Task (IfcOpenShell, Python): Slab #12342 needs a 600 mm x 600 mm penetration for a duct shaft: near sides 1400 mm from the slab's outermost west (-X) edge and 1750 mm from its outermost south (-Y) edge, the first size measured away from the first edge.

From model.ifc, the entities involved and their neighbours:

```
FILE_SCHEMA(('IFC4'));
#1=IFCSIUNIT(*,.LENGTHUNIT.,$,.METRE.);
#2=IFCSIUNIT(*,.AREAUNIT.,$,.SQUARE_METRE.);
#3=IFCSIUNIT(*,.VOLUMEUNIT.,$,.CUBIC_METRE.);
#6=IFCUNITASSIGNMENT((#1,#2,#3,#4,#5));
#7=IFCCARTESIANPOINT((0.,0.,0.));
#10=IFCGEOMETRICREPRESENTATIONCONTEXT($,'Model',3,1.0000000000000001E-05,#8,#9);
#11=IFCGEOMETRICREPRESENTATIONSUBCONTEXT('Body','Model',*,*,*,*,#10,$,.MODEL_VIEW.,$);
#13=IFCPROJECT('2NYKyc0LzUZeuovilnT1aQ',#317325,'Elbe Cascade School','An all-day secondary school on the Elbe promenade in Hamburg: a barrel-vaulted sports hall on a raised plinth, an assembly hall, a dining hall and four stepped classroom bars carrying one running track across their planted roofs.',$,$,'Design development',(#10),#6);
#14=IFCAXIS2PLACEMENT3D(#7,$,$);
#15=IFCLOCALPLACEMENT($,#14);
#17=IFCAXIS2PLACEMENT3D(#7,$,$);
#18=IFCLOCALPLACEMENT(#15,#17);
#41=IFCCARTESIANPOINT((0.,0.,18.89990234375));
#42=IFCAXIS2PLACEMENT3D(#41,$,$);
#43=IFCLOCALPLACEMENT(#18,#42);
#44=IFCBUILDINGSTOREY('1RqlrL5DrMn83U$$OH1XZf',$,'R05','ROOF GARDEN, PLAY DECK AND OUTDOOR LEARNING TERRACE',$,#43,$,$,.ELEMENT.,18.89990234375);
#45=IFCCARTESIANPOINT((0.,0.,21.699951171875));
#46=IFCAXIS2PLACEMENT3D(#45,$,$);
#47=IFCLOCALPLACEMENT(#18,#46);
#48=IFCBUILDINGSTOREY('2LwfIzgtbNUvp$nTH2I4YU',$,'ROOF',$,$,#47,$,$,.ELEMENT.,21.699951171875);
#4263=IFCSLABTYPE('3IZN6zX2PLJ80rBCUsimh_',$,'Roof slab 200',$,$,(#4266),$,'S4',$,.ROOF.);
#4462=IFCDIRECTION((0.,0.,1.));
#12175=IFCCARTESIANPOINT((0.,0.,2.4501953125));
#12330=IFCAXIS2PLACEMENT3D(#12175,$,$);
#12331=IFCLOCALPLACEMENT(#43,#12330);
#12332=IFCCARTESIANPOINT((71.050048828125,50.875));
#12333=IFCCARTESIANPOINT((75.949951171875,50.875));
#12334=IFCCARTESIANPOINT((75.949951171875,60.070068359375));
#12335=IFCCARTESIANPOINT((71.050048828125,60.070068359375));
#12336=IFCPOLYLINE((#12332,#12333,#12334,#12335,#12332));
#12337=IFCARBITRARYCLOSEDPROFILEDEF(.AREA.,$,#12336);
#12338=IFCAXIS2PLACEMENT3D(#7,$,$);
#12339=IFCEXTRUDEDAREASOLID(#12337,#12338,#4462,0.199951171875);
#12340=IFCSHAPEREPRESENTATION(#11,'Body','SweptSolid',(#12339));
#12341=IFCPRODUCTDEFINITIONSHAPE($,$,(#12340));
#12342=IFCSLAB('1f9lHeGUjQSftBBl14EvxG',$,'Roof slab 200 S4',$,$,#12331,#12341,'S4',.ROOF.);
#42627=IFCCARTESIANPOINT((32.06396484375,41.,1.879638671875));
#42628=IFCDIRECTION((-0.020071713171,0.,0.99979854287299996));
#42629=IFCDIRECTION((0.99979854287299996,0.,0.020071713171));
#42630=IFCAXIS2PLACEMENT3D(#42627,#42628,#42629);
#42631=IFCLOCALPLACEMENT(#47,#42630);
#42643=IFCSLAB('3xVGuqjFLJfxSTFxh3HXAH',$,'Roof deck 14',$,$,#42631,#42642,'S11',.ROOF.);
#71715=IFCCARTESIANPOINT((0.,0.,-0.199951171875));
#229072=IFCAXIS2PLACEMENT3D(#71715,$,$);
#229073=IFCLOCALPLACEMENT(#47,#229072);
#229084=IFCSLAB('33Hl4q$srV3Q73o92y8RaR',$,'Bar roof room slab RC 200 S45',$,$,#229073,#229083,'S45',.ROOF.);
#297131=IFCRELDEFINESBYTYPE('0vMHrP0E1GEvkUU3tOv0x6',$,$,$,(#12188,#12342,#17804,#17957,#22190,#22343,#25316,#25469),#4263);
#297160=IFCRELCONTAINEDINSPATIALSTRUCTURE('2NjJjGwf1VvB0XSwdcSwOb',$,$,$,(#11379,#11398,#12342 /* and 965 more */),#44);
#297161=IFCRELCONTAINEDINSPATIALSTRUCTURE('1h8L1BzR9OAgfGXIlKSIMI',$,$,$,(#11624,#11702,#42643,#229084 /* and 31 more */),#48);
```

```python
import numpy as np
import ifcopenshell
import ifcopenshell.api.feature
import ifcopenshell.api.geometry
import ifcopenshell.api.root
import ifcopenshell.geom
import ifcopenshell.util.placement
import ifcopenshell.util.representation
import ifcopenshell.util.shape
import ifcopenshell.util.unit

model = ifcopenshell.open("model.ifc")
unit_scale = ifcopenshell.util.unit.calculate_unit_scale(model)
settings = ifcopenshell.geom.settings()


def volume(element):
    """Net volume in cubic metres, openings subtracted."""
    shape = ifcopenshell.geom.create_shape(settings, element)
    return ifcopenshell.util.shape.get_volume(shape.geometry)


slab = model.by_guid("1f9lHeGUjQSftBBl14EvxG")
before = volume(slab)

# Extent in the slab's own axes, in metres. The edges named are its -X and -Y sides.
slab_shape = ifcopenshell.geom.create_shape(settings, slab)
vertices = ifcopenshell.util.shape.get_vertices(slab_shape.geometry)
x_min, y_min, bottom = vertices.min(axis=0)
top = vertices[:, 2].max()

opening = ifcopenshell.api.root.create_entity(model, ifc_class="IfcOpeningElement", name="Duct shaft opening", predefined_type="OPENING")
context = ifcopenshell.util.representation.get_context(model, "Model", "Body", "MODEL_VIEW")
width, depth = 0.6, 0.6
outline = [(0.0, 0.0), (width, 0.0), (width, depth), (0.0, depth), (0.0, 0.0)]
# Overshoot both faces by 50 mm so the cut is clean.
shape = ifcopenshell.api.geometry.add_slab_representation(
    model, context=context, depth=top - bottom + 0.1, polyline=outline
)
ifcopenshell.api.geometry.assign_representation(model, product=opening, representation=shape)

matrix = ifcopenshell.util.placement.get_local_placement(slab.ObjectPlacement)
matrix[:, 3] = matrix @ np.append(np.array([x_min + 1.4, y_min + 1.75, bottom - 0.05]) / unit_scale, 1.0)
ifcopenshell.api.geometry.edit_object_placement(model, product=opening, matrix=matrix, is_si=False)
ifcopenshell.api.feature.add_feature(model, feature=opening, element=slab)

after = volume(slab)

print(f"slab volume {before:.3f} -> {after:.3f} m3")

model.write("model_edited.ifc")
```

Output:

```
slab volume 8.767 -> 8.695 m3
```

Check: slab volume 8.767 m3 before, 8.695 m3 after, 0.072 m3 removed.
